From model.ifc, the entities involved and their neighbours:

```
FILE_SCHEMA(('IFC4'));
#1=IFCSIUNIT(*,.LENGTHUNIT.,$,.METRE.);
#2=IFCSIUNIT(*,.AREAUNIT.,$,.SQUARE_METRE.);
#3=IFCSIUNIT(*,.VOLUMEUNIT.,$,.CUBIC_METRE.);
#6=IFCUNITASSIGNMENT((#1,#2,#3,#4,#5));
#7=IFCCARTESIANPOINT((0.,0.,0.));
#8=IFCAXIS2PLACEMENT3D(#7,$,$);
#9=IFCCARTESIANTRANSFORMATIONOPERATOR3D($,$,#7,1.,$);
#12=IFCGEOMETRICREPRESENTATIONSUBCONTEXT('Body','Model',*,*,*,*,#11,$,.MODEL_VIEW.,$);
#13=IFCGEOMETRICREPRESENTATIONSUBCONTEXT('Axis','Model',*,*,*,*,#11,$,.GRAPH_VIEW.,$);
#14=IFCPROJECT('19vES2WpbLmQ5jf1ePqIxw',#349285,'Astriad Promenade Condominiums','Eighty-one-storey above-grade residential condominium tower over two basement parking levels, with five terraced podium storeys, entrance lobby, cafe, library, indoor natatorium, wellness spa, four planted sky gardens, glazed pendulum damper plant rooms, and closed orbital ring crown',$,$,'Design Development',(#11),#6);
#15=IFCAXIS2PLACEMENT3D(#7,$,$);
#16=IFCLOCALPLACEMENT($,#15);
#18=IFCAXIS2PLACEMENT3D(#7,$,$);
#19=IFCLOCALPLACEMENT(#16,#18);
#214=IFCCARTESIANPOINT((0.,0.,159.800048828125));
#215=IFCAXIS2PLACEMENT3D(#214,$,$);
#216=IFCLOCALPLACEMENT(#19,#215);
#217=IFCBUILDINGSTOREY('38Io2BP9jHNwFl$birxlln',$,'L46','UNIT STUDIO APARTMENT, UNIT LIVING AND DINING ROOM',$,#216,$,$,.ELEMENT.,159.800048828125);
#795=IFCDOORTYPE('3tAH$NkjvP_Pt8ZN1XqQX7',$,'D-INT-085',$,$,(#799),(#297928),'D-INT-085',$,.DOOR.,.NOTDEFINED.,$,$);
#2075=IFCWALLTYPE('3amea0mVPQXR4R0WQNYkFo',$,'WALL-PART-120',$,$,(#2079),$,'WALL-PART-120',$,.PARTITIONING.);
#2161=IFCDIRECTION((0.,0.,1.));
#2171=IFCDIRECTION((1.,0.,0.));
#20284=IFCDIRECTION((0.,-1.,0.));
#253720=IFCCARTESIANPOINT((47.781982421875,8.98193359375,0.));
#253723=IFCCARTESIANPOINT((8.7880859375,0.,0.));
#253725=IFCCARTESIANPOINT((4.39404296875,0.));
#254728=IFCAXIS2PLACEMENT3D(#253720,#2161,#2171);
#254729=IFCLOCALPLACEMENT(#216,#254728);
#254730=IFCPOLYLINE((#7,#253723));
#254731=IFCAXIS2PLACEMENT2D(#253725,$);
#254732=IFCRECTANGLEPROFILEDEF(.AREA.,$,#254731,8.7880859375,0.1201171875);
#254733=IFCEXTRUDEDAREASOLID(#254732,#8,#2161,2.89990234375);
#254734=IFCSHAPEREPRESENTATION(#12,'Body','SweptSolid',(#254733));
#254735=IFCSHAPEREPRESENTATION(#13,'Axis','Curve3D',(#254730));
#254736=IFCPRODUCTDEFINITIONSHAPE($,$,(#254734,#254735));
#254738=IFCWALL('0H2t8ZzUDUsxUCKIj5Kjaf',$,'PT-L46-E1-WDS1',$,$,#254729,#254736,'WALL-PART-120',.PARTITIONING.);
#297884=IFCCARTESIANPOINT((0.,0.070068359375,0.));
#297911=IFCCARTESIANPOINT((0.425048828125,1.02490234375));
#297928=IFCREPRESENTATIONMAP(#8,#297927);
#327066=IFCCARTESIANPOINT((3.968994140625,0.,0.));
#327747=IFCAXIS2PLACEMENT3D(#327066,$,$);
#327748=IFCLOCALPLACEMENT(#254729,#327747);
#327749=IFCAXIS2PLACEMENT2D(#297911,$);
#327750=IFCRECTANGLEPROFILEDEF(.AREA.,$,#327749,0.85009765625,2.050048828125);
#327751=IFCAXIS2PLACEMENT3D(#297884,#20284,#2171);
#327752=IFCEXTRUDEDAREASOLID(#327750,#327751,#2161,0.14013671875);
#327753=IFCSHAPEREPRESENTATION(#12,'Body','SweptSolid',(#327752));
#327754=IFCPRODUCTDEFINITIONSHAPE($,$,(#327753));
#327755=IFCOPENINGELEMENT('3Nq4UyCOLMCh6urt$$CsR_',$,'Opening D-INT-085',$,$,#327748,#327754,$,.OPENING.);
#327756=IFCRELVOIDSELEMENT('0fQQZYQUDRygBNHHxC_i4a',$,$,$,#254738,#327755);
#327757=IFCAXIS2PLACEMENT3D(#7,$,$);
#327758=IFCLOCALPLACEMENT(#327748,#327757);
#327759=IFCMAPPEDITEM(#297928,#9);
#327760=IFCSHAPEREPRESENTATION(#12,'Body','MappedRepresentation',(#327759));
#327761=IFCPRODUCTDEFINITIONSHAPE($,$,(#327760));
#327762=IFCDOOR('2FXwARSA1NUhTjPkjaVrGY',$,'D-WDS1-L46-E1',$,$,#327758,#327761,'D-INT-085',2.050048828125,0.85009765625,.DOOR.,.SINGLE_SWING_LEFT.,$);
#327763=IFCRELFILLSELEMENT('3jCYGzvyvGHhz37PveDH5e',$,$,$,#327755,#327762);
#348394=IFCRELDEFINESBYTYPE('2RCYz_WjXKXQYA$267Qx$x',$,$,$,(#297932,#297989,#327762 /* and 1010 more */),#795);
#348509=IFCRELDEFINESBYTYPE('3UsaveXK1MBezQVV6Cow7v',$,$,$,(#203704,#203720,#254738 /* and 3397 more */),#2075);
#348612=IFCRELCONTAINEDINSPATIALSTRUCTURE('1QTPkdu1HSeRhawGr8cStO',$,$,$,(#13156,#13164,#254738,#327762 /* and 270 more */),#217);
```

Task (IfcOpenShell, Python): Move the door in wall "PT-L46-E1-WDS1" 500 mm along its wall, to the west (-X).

```python
import ifcopenshell
import ifcopenshell.api.geometry
import ifcopenshell.util.placement
import ifcopenshell.util.unit

model = ifcopenshell.open("model.ifc")
unit_scale = ifcopenshell.util.unit.calculate_unit_scale(model)

door = model.by_guid("2FXwARSA1NUhTjPkjaVrGY")
opening = door.FillsVoids[0].RelatingOpeningElement
wall = opening.VoidsElements[0].RelatingBuildingElement

wall_matrix = ifcopenshell.util.placement.get_local_placement(wall.ObjectPlacement)
shift = wall_matrix[:3, 0] * -0.5 / unit_scale
before = ifcopenshell.util.placement.get_local_placement(door.ObjectPlacement)[:3, 3].copy()

# The door is placed relative to its opening, so it follows when the opening moves.
matrix = ifcopenshell.util.placement.get_local_placement(opening.ObjectPlacement)
matrix[:3, 3] += shift
ifcopenshell.api.geometry.edit_object_placement(
    model, product=opening, matrix=matrix, is_si=False, should_transform_children=True
)

after = ifcopenshell.util.placement.get_local_placement(door.ObjectPlacement)[:3, 3]
print("door moved by", (after - before).round(3) + 0.0)

model.write("model_edited.ifc")
```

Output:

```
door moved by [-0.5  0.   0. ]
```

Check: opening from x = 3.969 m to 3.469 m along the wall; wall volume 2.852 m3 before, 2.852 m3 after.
